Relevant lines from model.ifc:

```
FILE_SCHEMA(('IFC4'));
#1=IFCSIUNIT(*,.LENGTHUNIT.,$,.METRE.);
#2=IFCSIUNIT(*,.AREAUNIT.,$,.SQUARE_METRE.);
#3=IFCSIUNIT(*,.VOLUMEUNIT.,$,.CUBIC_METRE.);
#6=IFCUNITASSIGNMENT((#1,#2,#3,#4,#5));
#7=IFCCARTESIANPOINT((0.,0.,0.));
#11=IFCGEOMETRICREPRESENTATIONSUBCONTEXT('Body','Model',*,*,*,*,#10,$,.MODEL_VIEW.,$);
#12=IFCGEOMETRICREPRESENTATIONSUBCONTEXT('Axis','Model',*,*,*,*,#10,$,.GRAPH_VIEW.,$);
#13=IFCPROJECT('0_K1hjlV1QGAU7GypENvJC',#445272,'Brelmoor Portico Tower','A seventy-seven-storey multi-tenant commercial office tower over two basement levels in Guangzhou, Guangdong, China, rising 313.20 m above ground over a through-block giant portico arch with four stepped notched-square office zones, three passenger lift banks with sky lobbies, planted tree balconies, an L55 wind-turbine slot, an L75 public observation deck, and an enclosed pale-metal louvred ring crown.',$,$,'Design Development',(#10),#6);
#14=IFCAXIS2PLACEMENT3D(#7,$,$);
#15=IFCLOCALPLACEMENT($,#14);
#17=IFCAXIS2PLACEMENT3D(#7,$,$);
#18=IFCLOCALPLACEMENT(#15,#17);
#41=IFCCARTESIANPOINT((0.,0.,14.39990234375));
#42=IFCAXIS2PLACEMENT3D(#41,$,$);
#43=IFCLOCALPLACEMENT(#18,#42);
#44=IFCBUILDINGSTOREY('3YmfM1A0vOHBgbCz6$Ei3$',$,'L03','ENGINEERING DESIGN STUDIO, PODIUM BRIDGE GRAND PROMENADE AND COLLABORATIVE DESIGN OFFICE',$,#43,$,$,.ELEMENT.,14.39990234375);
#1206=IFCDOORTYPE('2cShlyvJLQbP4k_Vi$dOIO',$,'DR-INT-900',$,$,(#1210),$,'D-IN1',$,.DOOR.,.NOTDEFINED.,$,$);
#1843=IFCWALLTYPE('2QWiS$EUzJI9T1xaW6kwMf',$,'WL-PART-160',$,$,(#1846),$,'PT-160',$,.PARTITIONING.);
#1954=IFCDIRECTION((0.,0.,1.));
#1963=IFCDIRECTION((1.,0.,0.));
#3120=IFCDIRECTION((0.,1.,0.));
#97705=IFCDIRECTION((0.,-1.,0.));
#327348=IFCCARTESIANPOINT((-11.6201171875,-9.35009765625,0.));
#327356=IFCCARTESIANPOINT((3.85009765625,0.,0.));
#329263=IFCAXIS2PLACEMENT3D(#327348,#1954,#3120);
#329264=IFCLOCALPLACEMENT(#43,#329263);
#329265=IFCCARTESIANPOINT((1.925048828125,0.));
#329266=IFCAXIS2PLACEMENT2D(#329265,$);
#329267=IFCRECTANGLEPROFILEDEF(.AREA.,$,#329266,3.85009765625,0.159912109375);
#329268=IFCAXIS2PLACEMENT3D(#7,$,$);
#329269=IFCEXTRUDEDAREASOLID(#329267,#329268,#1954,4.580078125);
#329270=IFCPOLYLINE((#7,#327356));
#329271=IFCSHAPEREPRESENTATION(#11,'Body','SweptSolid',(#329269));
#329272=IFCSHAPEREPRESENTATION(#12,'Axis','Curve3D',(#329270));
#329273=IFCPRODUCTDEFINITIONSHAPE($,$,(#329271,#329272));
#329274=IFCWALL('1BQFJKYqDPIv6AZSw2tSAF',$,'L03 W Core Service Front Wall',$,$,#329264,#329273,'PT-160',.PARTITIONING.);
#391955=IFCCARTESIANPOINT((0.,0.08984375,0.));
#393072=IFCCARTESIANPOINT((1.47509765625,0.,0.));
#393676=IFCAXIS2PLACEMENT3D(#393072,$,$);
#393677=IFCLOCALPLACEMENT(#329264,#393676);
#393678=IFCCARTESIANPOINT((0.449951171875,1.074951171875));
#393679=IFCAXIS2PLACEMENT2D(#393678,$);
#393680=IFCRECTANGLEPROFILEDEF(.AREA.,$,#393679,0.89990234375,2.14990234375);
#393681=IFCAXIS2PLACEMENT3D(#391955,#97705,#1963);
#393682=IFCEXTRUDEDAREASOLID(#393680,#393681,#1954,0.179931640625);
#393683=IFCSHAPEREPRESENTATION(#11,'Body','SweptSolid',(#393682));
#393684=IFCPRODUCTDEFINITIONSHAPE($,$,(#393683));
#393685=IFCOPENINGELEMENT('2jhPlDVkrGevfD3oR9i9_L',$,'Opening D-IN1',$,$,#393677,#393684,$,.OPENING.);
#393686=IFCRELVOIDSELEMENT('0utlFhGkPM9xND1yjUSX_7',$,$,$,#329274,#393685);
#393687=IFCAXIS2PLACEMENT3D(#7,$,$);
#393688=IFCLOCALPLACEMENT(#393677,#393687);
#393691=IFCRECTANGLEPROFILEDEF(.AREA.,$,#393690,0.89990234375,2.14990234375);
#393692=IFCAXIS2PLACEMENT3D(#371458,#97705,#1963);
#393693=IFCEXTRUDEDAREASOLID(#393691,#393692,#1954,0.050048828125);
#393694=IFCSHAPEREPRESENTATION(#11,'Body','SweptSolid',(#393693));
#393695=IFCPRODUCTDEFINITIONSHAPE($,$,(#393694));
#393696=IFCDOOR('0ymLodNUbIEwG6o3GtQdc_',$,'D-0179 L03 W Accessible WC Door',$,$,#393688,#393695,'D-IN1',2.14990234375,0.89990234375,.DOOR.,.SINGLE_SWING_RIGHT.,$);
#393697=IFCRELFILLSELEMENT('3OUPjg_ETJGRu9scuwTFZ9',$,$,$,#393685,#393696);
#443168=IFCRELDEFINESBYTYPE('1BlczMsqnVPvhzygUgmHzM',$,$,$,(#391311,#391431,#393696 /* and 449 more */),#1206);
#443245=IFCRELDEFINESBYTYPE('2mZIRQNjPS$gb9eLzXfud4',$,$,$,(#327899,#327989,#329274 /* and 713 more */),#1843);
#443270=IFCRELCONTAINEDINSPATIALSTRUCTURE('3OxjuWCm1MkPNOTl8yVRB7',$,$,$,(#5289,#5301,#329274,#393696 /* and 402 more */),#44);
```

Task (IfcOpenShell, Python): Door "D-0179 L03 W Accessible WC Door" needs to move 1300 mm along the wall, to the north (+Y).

```python
import ifcopenshell
import ifcopenshell.api.geometry
import ifcopenshell.util.placement

model = ifcopenshell.open("model.ifc")

door = model.by_guid("0ymLodNUbIEwG6o3GtQdc_")
opening = door.FillsVoids[0].RelatingOpeningElement
wall = opening.VoidsElements[0].RelatingBuildingElement

wall_matrix = ifcopenshell.util.placement.get_local_placement(wall.ObjectPlacement)
shift = wall_matrix[:3, 0] * 1.3
before = ifcopenshell.util.placement.get_local_placement(door.ObjectPlacement)[:3, 3].copy()

# The door is placed relative to its opening, so it follows when the opening moves.
matrix = ifcopenshell.util.placement.get_local_placement(opening.ObjectPlacement)
matrix[:3, 3] += shift
ifcopenshell.api.geometry.edit_object_placement(
    model, product=opening, matrix=matrix, is_si=False, should_transform_children=True
)

after = ifcopenshell.util.placement.get_local_placement(door.ObjectPlacement)[:3, 3]
print("door moved by", (after - before).round(3) + 0.0)

model.write("model_edited.ifc")
```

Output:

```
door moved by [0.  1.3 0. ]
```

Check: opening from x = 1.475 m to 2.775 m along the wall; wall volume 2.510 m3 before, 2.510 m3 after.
